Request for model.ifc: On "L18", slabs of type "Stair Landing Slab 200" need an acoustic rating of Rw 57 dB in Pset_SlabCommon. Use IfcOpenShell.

First a look at what the model holds.

```python
import ifcopenshell
import ifcopenshell.util.element

model = ifcopenshell.open("model.ifc")
print(model.schema)
storey = next(s for s in model.by_type("IfcBuildingStorey") if s.Name == "L18")
slabs = [e for e in ifcopenshell.util.element.get_decomposition(storey) if e.is_a("IfcSlab")]
seen = {}
for e in slabs:
    element_type = ifcopenshell.util.element.get_type(e)
    key = (element_type.Name if element_type != e and element_type else None, ifcopenshell.util.element.get_pset(e, "Pset_SlabCommon", "AcousticRating"))
    seen[key] = seen.get(key, 0) + 1
for (name, value), count in sorted(seen.items(), key=str):
    print(count, "x", name, "|", value)
```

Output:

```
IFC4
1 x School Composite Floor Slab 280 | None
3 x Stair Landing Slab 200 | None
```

```python
import ifcopenshell
import ifcopenshell.api.pset
import ifcopenshell.util.element

model = ifcopenshell.open("model.ifc")

storey = next(s for s in model.by_type("IfcBuildingStorey") if s.Name == "L18")
slabs = [e for e in ifcopenshell.util.element.get_decomposition(storey) if e.is_a("IfcSlab")]

count = 0
for e in slabs:
    element_type = ifcopenshell.util.element.get_type(e)
    if element_type in (None, e) or element_type.Name != "Stair Landing Slab 200":
        continue
    found = ifcopenshell.util.element.get_pset(e, "Pset_SlabCommon", should_inherit=False)
    if found:
        pset = model.by_id(found["id"])
        if len(ifcopenshell.util.element.get_elements_by_pset(pset)) > 1:
            pset = ifcopenshell.api.pset.unshare_pset(model, products=[e], pset=pset)[0]
    else:
        pset = ifcopenshell.api.pset.add_pset(model, product=e, name="Pset_SlabCommon")
    ifcopenshell.api.pset.edit_pset(model, pset=pset, properties={"AcousticRating": "Rw 57 dB"})
    count += 1

print(count, "slabs updated")

model.write("model_v2.ifc")
```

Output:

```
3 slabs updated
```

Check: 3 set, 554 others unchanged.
